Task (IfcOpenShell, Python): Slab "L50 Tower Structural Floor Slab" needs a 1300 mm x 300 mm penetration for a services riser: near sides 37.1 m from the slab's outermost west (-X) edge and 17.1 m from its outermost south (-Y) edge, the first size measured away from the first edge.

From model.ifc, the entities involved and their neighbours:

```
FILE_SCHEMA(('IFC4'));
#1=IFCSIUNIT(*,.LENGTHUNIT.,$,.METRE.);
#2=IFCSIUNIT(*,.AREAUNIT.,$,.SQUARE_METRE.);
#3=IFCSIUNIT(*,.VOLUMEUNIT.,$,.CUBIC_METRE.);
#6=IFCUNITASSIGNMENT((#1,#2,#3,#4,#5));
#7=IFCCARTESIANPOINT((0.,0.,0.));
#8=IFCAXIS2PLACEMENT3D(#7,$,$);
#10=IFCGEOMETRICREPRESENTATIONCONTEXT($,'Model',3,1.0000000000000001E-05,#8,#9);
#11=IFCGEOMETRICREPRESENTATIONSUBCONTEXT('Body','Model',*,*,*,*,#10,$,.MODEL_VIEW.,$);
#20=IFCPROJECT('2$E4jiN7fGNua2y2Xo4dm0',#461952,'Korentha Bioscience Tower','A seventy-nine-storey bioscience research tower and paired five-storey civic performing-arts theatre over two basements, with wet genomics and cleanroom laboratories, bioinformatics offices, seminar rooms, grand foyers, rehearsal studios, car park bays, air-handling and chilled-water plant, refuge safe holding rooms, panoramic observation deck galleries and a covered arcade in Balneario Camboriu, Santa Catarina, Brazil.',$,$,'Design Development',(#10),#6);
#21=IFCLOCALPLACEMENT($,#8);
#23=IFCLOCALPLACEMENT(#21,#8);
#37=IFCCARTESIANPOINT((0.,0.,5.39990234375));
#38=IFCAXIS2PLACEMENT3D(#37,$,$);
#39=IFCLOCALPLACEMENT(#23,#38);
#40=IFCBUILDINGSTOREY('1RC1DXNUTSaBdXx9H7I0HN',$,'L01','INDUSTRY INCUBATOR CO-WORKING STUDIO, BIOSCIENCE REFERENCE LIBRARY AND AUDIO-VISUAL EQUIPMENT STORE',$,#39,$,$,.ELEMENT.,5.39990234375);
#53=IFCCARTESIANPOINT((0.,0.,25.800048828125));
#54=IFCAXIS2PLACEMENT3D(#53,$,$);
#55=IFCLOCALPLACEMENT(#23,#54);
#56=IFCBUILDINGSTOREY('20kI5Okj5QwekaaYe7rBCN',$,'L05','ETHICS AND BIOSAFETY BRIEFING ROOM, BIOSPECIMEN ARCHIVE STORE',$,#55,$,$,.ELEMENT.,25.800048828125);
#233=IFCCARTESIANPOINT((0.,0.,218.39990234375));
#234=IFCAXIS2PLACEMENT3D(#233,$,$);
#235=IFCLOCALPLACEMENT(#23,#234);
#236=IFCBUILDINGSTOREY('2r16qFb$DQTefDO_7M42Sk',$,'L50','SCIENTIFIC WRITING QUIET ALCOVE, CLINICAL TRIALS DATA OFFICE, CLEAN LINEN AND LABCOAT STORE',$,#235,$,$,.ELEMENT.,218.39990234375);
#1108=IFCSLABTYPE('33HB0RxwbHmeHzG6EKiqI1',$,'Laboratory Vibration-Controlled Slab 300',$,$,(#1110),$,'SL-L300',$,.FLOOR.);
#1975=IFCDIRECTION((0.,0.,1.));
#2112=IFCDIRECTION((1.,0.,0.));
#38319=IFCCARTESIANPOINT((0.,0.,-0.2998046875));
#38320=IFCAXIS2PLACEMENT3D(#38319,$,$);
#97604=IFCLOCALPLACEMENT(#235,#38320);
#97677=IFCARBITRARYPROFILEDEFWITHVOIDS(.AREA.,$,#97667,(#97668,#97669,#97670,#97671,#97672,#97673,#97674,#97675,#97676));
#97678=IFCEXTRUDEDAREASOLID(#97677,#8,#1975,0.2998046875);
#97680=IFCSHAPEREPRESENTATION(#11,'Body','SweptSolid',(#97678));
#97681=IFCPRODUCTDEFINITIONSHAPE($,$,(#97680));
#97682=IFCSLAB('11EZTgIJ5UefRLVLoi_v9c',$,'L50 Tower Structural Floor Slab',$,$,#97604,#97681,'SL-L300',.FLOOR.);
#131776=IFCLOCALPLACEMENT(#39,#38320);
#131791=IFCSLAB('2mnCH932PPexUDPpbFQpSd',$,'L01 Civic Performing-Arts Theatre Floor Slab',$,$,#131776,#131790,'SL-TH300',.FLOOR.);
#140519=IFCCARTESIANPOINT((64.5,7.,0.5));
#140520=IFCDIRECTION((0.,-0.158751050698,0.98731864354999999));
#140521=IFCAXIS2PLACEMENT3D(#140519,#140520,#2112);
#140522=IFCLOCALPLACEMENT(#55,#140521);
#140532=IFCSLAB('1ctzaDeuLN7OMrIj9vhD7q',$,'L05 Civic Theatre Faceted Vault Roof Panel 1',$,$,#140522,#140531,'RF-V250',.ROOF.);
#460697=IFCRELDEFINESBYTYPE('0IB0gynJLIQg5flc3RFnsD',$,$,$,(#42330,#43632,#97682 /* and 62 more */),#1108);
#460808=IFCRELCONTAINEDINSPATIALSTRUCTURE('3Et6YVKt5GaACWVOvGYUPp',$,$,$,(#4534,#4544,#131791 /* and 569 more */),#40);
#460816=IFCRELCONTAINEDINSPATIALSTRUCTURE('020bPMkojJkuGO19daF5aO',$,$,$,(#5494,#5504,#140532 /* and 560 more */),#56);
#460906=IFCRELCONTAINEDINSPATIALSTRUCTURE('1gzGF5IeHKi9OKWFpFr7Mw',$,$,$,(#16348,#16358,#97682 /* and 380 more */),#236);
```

```python
import numpy as np
import ifcopenshell
import ifcopenshell.api.feature
import ifcopenshell.api.geometry
import ifcopenshell.api.root
import ifcopenshell.geom
import ifcopenshell.util.placement
import ifcopenshell.util.representation
import ifcopenshell.util.shape
import ifcopenshell.util.unit

model = ifcopenshell.open("model.ifc")
unit_scale = ifcopenshell.util.unit.calculate_unit_scale(model)
settings = ifcopenshell.geom.settings()


def volume(element):
    """Net volume in cubic metres, openings subtracted."""
    shape = ifcopenshell.geom.create_shape(settings, element)
    return ifcopenshell.util.shape.get_volume(shape.geometry)


slab = model.by_guid("11EZTgIJ5UefRLVLoi_v9c")
before = volume(slab)

# Extent in the slab's own axes, in metres. The edges named are its -X and -Y sides.
slab_shape = ifcopenshell.geom.create_shape(settings, slab)
vertices = ifcopenshell.util.shape.get_vertices(slab_shape.geometry)
x_min, y_min, bottom = vertices.min(axis=0)
top = vertices[:, 2].max()

opening = ifcopenshell.api.root.create_entity(model, ifc_class="IfcOpeningElement", name="Services riser opening", predefined_type="OPENING")
context = ifcopenshell.util.representation.get_context(model, "Model", "Body", "MODEL_VIEW")
width, depth = 1.3, 0.3
outline = [(0.0, 0.0), (width, 0.0), (width, depth), (0.0, depth), (0.0, 0.0)]
# Overshoot both faces by 50 mm so the cut is clean.
shape = ifcopenshell.api.geometry.add_slab_representation(
    model, context=context, depth=top - bottom + 0.1, polyline=outline
)
ifcopenshell.api.geometry.assign_representation(model, product=opening, representation=shape)

matrix = ifcopenshell.util.placement.get_local_placement(slab.ObjectPlacement)
matrix[:, 3] = matrix @ np.append(np.array([x_min + 37.1, y_min + 17.1, bottom - 0.05]) / unit_scale, 1.0)
ifcopenshell.api.geometry.edit_object_placement(model, product=opening, matrix=matrix, is_si=False)
ifcopenshell.api.feature.add_feature(model, feature=opening, element=slab)

after = volume(slab)

print(f"slab volume {before:.3f} -> {after:.3f} m3")

model.write("model_rev.ifc")
```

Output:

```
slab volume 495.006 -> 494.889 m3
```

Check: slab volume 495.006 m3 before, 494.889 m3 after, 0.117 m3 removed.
